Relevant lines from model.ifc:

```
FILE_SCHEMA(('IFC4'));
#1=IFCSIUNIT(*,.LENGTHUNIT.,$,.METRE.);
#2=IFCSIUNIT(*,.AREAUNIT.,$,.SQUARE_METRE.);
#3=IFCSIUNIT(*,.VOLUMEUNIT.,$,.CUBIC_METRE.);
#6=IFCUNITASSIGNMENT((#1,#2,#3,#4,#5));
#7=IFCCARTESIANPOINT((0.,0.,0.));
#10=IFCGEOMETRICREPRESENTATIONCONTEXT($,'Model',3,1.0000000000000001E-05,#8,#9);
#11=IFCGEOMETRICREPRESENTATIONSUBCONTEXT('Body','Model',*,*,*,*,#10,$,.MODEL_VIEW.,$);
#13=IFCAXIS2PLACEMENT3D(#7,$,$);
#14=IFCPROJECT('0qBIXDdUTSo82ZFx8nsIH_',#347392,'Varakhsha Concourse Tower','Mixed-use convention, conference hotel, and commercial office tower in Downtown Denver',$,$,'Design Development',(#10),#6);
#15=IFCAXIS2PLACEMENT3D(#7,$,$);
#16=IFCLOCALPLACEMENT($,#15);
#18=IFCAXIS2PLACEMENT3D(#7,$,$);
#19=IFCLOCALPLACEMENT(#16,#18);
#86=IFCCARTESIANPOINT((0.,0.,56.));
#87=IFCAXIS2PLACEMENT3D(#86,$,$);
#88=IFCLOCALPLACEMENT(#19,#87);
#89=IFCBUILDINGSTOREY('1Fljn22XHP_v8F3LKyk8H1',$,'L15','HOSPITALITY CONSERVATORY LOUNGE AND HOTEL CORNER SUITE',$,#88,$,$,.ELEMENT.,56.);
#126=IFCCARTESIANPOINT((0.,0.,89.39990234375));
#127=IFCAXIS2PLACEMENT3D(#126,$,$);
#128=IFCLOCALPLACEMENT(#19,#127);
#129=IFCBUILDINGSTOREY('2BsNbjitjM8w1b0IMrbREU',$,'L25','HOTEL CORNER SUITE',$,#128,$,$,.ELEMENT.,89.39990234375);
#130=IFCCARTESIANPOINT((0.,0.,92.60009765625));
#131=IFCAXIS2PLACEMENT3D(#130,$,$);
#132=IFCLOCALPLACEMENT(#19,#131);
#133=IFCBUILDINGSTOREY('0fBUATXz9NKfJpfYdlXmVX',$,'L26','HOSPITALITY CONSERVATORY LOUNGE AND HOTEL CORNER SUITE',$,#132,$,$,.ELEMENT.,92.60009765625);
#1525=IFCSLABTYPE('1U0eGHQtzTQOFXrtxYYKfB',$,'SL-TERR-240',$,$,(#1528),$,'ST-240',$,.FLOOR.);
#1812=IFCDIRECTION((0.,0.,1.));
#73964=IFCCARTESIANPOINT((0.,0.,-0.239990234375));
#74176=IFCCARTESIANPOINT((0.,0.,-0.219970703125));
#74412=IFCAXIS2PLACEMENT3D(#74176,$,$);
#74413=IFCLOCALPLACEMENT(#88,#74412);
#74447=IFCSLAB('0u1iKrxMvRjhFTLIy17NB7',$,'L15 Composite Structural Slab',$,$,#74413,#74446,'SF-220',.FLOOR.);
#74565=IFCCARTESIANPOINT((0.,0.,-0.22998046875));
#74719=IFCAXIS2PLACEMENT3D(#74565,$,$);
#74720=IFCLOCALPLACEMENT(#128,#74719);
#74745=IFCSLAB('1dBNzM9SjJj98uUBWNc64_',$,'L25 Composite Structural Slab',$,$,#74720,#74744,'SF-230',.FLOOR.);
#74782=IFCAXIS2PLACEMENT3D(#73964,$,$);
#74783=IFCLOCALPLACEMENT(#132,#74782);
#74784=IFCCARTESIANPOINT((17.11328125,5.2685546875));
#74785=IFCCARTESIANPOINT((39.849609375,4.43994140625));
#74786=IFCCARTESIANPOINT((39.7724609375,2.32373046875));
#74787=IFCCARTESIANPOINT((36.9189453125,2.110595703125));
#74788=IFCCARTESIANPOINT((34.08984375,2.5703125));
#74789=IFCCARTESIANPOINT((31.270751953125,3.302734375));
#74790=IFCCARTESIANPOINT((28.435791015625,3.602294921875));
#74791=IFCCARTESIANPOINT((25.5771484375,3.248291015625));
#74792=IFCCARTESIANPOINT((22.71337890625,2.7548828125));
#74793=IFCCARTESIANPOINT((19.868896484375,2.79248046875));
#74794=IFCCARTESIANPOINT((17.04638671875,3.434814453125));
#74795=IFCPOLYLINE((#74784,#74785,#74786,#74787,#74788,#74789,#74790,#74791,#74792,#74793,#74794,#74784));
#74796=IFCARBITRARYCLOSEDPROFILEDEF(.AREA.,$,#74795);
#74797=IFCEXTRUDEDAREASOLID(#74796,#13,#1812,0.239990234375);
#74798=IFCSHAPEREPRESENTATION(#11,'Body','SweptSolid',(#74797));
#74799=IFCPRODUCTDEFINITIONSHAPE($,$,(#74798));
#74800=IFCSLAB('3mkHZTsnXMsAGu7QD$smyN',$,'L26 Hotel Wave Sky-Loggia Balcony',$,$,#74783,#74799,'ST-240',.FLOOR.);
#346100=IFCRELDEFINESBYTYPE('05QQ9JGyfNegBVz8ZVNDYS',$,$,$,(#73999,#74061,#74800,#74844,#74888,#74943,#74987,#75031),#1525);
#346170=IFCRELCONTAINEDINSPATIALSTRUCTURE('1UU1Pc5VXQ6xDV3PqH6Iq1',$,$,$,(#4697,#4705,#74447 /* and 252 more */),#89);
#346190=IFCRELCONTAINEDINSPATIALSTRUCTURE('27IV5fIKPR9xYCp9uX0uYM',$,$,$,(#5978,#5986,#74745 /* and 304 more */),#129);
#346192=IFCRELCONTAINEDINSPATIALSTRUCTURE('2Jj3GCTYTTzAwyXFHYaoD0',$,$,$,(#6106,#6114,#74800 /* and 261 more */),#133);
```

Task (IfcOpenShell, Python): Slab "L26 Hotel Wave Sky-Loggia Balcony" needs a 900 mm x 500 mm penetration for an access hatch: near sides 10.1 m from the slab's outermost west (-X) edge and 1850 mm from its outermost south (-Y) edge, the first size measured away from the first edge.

```python
import numpy as np
import ifcopenshell
import ifcopenshell.api.feature
import ifcopenshell.api.geometry
import ifcopenshell.api.root
import ifcopenshell.geom
import ifcopenshell.util.placement
import ifcopenshell.util.representation
import ifcopenshell.util.shape
import ifcopenshell.util.unit

model = ifcopenshell.open("model.ifc")
unit_scale = ifcopenshell.util.unit.calculate_unit_scale(model)
settings = ifcopenshell.geom.settings()


def volume(element):
    """Net volume in cubic metres, openings subtracted."""
    shape = ifcopenshell.geom.create_shape(settings, element)
    return ifcopenshell.util.shape.get_volume(shape.geometry)


slab = model.by_id(74800)
before = volume(slab)

# Extent in the slab's own axes, in metres. The edges named are its -X and -Y sides.
slab_shape = ifcopenshell.geom.create_shape(settings, slab)
vertices = ifcopenshell.util.shape.get_vertices(slab_shape.geometry)
x_min, y_min, bottom = vertices.min(axis=0)
top = vertices[:, 2].max()

opening = ifcopenshell.api.root.create_entity(model, ifc_class="IfcOpeningElement", name="Access hatch opening", predefined_type="OPENING")
context = ifcopenshell.util.representation.get_context(model, "Model", "Body", "MODEL_VIEW")
width, depth = 0.9, 0.5
outline = [(0.0, 0.0), (width, 0.0), (width, depth), (0.0, depth), (0.0, 0.0)]
# Overshoot both faces by 50 mm so the cut is clean.
shape = ifcopenshell.api.geometry.add_slab_representation(
    model, context=context, depth=top - bottom + 0.1, polyline=outline
)
ifcopenshell.api.geometry.assign_representation(model, product=opening, representation=shape)

matrix = ifcopenshell.util.placement.get_local_placement(slab.ObjectPlacement)
matrix[:, 3] = matrix @ np.append(np.array([x_min + 10.1, y_min + 1.85, bottom - 0.05]) / unit_scale, 1.0)
ifcopenshell.api.geometry.edit_object_placement(model, product=opening, matrix=matrix, is_si=False)
ifcopenshell.api.feature.add_feature(model, feature=opening, element=slab)

after = volume(slab)

print(f"slab volume {before:.3f} -> {after:.3f} m3")

model.write("model_edited.ifc")
```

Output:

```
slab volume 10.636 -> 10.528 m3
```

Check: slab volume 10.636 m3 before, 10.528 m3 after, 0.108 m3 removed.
